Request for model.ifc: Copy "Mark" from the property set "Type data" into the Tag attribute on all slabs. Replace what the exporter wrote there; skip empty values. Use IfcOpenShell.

First a look at what the model holds.

```python
import ifcopenshell
import ifcopenshell.util.element

model = ifcopenshell.open("model.ifc")
print(model.schema)
slabs = model.by_type("IfcSlab")
print(len(slabs), "slabs")
for e in slabs[:8]:
    source = ifcopenshell.util.element.get_pset(e, "Type data", "Mark")
    target = e.Tag
    print(e.id(), repr(source), repr(target), sep=" | ")
```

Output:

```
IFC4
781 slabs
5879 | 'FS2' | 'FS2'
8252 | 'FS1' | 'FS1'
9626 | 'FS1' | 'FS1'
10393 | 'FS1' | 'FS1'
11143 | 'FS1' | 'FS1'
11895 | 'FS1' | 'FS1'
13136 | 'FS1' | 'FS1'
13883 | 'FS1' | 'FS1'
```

```python
import ifcopenshell
import ifcopenshell.util.element

model = ifcopenshell.open("model.ifc")

count = 0
for e in model.by_type("IfcSlab"):
    value = ifcopenshell.util.element.get_pset(e, "Type data", "Mark")
    current = e.Tag
    if not value or not value.strip() or current == value:
        continue
    e.Tag = value
    count += 1

print(count, "slabs updated")

model.write("model-out.ifc")
```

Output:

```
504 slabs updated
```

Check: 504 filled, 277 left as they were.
